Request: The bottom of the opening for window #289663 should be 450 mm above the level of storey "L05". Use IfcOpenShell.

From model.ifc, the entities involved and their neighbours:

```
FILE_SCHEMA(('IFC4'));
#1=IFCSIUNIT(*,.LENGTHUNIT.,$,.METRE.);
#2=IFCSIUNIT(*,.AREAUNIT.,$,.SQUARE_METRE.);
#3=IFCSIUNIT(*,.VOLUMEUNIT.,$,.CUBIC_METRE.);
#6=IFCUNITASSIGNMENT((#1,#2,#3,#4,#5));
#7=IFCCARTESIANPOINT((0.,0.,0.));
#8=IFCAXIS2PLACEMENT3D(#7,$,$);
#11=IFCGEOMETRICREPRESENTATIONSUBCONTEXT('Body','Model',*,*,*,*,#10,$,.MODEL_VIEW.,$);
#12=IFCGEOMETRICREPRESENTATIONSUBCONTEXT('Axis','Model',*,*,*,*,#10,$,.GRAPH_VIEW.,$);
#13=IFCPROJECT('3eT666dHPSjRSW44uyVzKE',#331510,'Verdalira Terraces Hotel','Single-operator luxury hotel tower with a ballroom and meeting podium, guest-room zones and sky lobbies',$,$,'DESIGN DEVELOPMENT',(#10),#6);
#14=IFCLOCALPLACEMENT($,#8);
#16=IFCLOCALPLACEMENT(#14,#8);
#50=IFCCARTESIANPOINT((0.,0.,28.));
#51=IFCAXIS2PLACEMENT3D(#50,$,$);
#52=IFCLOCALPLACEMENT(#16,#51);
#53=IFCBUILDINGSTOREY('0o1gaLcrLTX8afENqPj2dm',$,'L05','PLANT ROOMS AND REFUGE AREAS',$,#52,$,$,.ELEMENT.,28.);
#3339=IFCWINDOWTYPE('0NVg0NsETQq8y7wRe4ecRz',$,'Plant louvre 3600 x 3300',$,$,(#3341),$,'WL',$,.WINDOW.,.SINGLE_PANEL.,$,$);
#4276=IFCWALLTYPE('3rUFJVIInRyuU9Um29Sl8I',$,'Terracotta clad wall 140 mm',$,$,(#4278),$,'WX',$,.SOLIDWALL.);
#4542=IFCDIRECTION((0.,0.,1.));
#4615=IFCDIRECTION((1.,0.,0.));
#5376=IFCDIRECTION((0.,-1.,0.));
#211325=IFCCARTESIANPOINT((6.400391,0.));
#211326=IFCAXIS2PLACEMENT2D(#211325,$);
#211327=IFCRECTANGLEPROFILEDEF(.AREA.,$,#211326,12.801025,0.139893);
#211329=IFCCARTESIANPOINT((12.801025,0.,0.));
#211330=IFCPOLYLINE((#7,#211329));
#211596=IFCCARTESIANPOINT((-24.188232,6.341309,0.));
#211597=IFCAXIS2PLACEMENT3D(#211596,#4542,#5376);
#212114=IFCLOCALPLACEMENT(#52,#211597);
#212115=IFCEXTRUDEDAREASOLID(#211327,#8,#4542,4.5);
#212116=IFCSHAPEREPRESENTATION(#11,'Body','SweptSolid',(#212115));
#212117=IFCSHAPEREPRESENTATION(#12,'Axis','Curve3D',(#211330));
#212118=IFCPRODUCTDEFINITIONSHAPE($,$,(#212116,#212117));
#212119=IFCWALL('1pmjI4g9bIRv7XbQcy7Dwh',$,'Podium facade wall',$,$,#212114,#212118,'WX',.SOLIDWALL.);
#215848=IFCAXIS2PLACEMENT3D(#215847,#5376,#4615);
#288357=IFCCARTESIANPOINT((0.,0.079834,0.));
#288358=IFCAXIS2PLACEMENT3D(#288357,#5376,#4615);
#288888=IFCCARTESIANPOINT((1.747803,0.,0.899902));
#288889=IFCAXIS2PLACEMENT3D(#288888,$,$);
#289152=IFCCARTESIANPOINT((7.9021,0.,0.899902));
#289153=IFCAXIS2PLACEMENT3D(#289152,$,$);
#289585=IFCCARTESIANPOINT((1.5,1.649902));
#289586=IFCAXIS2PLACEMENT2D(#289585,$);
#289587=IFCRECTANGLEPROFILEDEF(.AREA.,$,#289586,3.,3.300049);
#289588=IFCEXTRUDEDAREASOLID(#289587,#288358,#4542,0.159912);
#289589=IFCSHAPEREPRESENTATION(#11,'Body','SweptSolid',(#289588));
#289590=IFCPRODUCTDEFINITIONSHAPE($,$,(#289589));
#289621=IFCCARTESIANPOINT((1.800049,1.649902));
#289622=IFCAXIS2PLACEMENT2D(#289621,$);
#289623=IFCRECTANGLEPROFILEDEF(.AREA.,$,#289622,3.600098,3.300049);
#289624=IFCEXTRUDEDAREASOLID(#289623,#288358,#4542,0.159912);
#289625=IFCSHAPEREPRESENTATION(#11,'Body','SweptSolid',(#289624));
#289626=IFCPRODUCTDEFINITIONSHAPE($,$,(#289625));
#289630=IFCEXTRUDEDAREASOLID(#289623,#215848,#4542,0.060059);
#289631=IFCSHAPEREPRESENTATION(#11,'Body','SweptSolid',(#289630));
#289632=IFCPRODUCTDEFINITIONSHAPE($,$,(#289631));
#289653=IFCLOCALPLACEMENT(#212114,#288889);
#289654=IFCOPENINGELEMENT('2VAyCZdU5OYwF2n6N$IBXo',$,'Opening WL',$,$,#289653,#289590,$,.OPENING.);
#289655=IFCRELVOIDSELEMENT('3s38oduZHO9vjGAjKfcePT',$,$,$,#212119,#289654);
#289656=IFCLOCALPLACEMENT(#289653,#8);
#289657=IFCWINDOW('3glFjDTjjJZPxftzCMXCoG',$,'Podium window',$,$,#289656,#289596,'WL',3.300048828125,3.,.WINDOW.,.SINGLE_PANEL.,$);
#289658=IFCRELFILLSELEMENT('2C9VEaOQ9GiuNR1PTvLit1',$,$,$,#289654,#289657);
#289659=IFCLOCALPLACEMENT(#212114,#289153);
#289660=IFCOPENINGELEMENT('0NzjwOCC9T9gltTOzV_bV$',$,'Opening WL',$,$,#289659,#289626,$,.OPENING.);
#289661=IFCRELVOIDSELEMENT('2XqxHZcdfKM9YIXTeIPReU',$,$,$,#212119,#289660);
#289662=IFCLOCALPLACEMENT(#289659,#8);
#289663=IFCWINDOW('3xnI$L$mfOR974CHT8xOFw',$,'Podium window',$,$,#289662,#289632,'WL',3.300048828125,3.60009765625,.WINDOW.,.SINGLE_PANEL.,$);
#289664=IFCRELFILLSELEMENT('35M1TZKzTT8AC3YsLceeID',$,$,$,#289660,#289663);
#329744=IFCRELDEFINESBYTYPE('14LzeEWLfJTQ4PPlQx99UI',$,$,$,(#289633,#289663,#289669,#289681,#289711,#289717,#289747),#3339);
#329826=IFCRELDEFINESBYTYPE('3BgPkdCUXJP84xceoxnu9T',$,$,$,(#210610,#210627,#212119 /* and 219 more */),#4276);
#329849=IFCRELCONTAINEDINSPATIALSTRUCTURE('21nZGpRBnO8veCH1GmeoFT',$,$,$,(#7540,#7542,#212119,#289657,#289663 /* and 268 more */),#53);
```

```python
import numpy as np
import ifcopenshell
import ifcopenshell.api.geometry
import ifcopenshell.geom
import ifcopenshell.util.element
import ifcopenshell.util.placement
import ifcopenshell.util.shape
import ifcopenshell.util.unit

model = ifcopenshell.open("model.ifc")
unit_scale = ifcopenshell.util.unit.calculate_unit_scale(model)

window = model.by_guid("3xnI$L$mfOR974CHT8xOFw")
opening = window.FillsVoids[0].RelatingOpeningElement
storey = ifcopenshell.util.element.get_container(window, ifc_class="IfcBuildingStorey")
level = ifcopenshell.util.placement.get_local_placement(storey.ObjectPlacement)[2, 3]

# The opening's origin need not be at the sill, so measure its lowest point.
shape = ifcopenshell.geom.create_shape(ifcopenshell.geom.settings(), opening)
bottom = ifcopenshell.util.shape.get_shape_bottom_elevation(shape, shape.geometry) / unit_scale
dz = level + 0.45 / unit_scale - bottom

shift = np.array([0.0, 0.0, dz])
# The window is placed relative to its opening, so it follows when the opening moves.
matrix = ifcopenshell.util.placement.get_local_placement(opening.ObjectPlacement)
matrix[:3, 3] += shift
ifcopenshell.api.geometry.edit_object_placement(
    model, product=opening, matrix=matrix, is_si=False, should_transform_children=True
)

print(f"moved by {dz * unit_scale:+.3f} m")

model.write("model_edited.ifc")
```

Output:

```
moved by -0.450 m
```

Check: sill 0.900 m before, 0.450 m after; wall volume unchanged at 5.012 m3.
